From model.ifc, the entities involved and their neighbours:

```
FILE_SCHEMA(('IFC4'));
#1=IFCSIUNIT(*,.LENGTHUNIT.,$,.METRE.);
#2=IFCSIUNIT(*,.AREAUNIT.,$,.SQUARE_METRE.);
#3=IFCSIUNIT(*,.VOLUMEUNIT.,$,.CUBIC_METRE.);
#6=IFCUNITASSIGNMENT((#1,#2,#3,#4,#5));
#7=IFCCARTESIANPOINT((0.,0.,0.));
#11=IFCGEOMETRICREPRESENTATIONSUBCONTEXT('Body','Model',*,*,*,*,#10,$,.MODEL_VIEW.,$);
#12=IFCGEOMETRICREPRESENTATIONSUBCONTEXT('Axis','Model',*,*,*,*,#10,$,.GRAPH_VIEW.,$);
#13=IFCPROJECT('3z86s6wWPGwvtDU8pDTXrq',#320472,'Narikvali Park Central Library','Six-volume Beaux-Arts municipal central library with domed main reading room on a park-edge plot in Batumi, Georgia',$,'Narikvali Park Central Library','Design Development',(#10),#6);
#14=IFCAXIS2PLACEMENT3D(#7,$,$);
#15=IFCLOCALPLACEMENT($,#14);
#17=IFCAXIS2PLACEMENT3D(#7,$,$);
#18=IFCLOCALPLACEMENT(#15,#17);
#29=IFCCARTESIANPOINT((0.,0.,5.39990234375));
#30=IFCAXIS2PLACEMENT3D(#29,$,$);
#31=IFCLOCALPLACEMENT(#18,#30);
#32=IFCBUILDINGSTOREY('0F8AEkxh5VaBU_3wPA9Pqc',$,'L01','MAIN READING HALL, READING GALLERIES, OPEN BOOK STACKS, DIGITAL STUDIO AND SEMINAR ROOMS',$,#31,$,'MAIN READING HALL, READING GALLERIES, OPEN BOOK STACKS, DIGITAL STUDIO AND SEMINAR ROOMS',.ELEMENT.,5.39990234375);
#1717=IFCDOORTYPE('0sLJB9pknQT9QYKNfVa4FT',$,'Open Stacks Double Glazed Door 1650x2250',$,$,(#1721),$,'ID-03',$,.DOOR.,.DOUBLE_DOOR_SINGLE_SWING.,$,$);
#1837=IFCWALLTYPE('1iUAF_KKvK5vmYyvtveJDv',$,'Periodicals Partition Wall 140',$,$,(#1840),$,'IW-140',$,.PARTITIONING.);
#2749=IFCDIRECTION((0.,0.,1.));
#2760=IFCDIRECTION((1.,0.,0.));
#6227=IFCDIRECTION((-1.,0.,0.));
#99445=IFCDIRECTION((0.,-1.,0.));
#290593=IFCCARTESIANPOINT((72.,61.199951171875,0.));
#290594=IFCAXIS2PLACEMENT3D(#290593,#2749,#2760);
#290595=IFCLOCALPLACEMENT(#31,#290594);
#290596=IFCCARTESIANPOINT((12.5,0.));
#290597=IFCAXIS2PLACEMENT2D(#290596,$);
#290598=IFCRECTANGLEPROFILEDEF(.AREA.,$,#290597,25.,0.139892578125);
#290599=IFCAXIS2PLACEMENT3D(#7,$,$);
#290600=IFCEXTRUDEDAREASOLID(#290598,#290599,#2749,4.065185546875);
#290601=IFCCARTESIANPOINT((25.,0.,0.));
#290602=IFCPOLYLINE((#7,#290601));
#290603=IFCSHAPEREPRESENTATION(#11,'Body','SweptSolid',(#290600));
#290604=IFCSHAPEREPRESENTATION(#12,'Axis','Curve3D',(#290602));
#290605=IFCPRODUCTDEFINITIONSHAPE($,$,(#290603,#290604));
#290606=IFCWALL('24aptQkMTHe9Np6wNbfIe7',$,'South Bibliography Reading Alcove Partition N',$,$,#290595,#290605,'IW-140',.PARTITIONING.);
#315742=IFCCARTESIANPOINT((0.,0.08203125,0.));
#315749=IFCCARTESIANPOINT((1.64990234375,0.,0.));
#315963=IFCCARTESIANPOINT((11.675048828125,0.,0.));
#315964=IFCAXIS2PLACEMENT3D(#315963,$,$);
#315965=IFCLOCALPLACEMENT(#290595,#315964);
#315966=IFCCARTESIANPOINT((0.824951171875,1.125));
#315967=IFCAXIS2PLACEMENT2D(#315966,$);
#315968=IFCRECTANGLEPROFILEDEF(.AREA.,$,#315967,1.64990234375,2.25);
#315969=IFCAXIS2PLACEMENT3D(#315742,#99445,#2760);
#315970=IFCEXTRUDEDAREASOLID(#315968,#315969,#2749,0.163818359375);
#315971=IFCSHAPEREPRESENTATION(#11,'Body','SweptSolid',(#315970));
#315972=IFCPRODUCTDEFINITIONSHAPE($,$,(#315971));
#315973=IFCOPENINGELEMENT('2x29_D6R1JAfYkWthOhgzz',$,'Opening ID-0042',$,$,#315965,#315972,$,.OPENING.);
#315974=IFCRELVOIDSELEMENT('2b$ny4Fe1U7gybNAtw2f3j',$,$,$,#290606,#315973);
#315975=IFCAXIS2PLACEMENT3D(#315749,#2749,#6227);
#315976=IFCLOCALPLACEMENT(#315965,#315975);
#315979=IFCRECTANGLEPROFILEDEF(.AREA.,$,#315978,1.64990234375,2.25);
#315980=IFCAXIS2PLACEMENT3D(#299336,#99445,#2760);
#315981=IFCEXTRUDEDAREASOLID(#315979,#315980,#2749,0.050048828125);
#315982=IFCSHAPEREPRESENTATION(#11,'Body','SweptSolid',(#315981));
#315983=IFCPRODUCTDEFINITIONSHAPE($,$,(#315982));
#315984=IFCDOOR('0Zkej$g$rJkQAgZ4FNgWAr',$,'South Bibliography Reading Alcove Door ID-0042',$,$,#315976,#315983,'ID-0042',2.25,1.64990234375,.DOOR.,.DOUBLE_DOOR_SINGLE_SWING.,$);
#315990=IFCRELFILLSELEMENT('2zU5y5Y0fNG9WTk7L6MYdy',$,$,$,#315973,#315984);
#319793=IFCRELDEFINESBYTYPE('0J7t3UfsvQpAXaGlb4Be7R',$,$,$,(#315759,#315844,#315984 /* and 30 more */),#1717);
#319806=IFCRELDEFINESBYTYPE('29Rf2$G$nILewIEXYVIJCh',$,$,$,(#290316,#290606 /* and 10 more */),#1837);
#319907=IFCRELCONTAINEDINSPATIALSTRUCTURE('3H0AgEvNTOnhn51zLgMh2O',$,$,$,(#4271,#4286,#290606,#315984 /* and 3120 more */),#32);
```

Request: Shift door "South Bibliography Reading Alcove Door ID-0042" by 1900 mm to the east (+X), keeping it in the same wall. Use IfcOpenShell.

```python
import ifcopenshell
import ifcopenshell.api.geometry
import ifcopenshell.util.placement

model = ifcopenshell.open("model.ifc")

door = model.by_guid("0Zkej$g$rJkQAgZ4FNgWAr")
opening = door.FillsVoids[0].RelatingOpeningElement
wall = opening.VoidsElements[0].RelatingBuildingElement

wall_matrix = ifcopenshell.util.placement.get_local_placement(wall.ObjectPlacement)
shift = wall_matrix[:3, 0] * 1.9
before = ifcopenshell.util.placement.get_local_placement(door.ObjectPlacement)[:3, 3].copy()

# The door is placed relative to its opening, so it follows when the opening moves.
matrix = ifcopenshell.util.placement.get_local_placement(opening.ObjectPlacement)
matrix[:3, 3] += shift
ifcopenshell.api.geometry.edit_object_placement(
    model, product=opening, matrix=matrix, is_si=False, should_transform_children=True
)

after = ifcopenshell.util.placement.get_local_placement(door.ObjectPlacement)[:3, 3]
print("door moved by", (after - before).round(3) + 0.0)

model.write("model_updated.ifc")
```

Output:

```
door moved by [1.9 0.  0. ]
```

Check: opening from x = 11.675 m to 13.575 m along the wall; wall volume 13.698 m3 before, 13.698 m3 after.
